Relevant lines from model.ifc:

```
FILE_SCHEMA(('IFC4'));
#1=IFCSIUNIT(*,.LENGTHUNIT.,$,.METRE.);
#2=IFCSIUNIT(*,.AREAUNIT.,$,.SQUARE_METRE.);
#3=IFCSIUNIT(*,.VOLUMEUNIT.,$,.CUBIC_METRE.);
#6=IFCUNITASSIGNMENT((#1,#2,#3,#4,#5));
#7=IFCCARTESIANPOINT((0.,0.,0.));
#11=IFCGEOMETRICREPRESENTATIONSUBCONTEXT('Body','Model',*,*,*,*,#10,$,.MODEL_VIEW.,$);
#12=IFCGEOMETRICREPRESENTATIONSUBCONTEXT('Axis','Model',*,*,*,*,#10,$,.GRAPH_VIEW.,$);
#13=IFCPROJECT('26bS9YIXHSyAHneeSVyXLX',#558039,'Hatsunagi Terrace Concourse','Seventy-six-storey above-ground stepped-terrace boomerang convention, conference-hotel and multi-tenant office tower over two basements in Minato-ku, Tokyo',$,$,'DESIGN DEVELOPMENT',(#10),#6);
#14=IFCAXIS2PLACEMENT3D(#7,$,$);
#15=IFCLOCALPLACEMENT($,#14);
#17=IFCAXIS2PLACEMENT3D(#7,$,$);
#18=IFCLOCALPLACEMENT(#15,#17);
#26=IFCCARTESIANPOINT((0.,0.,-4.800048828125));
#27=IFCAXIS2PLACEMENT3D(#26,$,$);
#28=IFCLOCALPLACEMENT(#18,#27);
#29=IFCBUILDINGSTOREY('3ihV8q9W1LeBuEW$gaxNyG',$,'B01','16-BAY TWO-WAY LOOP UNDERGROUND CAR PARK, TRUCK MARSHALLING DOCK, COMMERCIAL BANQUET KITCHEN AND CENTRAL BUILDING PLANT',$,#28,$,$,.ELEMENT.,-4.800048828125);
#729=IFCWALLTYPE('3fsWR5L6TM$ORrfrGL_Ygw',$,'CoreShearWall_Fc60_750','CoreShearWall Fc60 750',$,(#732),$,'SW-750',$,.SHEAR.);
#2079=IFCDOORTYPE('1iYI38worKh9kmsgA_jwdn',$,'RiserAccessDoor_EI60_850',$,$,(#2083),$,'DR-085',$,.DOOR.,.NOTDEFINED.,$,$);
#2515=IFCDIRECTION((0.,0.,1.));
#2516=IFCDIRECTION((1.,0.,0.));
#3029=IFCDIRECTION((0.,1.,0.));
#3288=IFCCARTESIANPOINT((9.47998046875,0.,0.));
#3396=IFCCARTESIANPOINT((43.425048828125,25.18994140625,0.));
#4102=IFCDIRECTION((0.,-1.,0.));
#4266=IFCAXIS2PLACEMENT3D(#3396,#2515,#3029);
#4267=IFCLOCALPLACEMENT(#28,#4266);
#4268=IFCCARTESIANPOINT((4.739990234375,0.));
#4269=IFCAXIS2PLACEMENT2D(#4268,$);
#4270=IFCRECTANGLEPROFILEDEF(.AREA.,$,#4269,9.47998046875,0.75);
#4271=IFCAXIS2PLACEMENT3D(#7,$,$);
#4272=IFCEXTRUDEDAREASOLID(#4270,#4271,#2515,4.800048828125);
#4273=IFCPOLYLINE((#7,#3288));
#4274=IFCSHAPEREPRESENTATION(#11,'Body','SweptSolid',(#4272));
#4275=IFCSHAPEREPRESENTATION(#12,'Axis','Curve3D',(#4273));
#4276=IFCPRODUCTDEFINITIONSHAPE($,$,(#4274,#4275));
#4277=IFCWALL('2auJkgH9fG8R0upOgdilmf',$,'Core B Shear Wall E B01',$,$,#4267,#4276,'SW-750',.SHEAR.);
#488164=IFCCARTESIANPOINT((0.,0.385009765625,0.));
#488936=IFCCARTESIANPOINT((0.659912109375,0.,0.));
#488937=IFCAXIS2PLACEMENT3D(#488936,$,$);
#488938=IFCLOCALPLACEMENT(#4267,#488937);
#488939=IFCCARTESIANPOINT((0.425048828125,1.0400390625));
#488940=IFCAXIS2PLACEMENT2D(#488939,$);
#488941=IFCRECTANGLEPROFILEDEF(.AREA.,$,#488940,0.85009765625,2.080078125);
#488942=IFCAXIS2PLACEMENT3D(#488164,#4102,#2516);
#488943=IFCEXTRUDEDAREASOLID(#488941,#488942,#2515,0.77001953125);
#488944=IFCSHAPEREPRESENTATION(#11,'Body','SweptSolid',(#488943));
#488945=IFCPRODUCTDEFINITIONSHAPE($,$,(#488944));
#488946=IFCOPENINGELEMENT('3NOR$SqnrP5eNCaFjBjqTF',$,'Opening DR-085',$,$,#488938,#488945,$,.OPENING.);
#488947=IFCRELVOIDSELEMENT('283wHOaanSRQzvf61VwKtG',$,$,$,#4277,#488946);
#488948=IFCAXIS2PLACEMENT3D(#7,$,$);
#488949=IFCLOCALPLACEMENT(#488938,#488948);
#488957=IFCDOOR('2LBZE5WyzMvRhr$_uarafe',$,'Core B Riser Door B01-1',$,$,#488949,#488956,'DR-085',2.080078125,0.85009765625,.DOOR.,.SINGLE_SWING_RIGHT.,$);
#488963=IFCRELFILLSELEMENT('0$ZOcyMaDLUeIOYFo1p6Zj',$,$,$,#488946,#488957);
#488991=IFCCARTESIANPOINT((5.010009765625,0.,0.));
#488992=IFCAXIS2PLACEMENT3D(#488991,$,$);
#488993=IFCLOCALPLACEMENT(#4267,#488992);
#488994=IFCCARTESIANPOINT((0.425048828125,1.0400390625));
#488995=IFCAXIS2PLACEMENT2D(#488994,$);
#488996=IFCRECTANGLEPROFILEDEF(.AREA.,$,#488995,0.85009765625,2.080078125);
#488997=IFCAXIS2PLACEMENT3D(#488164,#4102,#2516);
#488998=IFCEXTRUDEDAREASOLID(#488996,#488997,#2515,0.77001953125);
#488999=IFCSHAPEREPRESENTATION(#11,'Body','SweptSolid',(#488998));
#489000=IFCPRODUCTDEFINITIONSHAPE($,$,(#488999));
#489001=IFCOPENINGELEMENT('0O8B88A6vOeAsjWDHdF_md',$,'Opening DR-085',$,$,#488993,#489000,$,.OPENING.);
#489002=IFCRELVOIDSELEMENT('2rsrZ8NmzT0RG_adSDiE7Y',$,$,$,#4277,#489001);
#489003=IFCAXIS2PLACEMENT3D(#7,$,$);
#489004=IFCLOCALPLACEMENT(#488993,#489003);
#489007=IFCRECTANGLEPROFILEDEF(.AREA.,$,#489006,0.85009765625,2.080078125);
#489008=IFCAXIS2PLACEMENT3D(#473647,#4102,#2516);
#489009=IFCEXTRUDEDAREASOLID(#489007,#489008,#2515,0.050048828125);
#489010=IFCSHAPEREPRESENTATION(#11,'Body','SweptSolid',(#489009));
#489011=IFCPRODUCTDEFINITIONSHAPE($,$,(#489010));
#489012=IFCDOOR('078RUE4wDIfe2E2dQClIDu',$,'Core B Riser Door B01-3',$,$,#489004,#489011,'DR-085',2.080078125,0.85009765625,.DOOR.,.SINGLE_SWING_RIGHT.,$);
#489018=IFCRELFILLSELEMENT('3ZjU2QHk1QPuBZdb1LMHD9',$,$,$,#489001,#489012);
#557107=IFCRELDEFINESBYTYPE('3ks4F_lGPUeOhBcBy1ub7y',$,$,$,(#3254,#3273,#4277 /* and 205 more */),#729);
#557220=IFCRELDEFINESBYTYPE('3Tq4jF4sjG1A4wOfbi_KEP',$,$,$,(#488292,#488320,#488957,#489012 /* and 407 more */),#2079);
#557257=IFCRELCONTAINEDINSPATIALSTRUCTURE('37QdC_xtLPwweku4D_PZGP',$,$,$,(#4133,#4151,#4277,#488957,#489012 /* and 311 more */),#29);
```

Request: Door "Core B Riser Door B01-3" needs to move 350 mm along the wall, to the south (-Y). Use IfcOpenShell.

```python
import ifcopenshell
import ifcopenshell.api.geometry
import ifcopenshell.util.placement

model = ifcopenshell.open("model.ifc")

door = model.by_guid("078RUE4wDIfe2E2dQClIDu")
opening = door.FillsVoids[0].RelatingOpeningElement
wall = opening.VoidsElements[0].RelatingBuildingElement

wall_matrix = ifcopenshell.util.placement.get_local_placement(wall.ObjectPlacement)
shift = wall_matrix[:3, 0] * -0.35
before = ifcopenshell.util.placement.get_local_placement(door.ObjectPlacement)[:3, 3].copy()

# The door is placed relative to its opening, so it follows when the opening moves.
matrix = ifcopenshell.util.placement.get_local_placement(opening.ObjectPlacement)
matrix[:3, 3] += shift
ifcopenshell.api.geometry.edit_object_placement(
    model, product=opening, matrix=matrix, is_si=False, should_transform_children=True
)

after = ifcopenshell.util.placement.get_local_placement(door.ObjectPlacement)[:3, 3]
print("door moved by", (after - before).round(3) + 0.0)

model.write("model_updated.ifc")
```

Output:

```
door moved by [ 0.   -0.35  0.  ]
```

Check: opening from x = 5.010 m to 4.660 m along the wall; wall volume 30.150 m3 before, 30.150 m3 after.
